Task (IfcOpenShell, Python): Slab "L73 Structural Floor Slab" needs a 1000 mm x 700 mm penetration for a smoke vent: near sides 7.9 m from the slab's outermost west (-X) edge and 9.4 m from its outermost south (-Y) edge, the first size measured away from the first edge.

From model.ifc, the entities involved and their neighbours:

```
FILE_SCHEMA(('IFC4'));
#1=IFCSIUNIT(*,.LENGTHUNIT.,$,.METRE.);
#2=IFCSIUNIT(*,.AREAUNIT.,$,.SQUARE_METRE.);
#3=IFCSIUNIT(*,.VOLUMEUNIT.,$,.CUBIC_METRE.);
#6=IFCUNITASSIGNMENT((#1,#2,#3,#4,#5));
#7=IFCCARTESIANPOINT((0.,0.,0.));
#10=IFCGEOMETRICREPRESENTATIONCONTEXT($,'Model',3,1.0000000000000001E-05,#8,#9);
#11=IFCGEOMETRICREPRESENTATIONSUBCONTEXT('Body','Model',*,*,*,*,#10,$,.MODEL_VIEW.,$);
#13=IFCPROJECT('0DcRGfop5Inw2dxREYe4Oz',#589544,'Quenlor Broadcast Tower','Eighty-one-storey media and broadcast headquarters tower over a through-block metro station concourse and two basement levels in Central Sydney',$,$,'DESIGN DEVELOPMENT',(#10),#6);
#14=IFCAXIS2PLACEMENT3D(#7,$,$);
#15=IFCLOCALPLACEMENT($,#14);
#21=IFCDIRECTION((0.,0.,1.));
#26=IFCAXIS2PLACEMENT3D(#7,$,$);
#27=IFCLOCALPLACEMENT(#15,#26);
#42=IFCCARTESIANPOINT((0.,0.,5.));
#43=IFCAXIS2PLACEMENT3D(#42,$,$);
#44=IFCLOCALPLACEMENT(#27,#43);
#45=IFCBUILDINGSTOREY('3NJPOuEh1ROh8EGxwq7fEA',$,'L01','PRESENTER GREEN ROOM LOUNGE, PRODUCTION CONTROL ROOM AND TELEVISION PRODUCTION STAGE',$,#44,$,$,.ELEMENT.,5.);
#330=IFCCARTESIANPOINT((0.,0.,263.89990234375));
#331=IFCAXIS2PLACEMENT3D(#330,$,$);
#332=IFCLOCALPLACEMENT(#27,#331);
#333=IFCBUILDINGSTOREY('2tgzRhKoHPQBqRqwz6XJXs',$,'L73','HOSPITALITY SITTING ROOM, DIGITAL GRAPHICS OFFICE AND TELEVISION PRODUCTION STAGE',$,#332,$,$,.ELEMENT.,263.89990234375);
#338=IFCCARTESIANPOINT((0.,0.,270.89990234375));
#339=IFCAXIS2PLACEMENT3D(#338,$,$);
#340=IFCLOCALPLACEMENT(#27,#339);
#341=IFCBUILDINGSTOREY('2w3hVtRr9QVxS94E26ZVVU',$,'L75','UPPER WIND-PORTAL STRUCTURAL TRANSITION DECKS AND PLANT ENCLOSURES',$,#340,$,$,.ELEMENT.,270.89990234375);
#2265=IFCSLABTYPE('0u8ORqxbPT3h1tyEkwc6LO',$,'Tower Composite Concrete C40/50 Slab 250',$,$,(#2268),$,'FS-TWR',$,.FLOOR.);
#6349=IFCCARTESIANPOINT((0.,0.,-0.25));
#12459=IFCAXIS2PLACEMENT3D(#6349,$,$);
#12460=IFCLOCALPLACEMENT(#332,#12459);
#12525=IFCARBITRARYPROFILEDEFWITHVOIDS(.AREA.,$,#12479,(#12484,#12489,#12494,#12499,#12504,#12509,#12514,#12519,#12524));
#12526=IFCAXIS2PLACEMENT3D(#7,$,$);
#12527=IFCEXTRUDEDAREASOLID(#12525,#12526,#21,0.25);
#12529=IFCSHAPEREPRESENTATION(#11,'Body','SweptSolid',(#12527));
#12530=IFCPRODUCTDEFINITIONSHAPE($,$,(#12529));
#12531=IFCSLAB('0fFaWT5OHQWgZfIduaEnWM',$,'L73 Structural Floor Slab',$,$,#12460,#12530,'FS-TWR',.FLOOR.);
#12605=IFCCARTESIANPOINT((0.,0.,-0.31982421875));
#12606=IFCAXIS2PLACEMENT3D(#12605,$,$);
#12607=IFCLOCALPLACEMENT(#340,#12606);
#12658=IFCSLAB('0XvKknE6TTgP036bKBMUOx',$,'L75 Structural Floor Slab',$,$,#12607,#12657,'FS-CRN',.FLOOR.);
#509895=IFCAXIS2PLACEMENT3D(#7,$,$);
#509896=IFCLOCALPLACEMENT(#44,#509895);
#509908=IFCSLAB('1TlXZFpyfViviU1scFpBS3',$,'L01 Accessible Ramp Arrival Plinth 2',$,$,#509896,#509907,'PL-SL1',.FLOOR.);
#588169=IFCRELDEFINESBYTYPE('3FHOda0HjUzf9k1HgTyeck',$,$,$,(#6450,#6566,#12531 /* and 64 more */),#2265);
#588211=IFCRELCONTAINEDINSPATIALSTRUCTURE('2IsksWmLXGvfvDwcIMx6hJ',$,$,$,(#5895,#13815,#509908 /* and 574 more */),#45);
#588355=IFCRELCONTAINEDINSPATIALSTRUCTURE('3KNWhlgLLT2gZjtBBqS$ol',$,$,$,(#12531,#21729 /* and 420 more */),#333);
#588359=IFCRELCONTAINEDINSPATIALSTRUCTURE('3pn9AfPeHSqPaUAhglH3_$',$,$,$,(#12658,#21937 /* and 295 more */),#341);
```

```python
import numpy as np
import ifcopenshell
import ifcopenshell.api.feature
import ifcopenshell.api.geometry
import ifcopenshell.api.root
import ifcopenshell.geom
import ifcopenshell.util.placement
import ifcopenshell.util.representation
import ifcopenshell.util.shape
import ifcopenshell.util.unit

model = ifcopenshell.open("model.ifc")
unit_scale = ifcopenshell.util.unit.calculate_unit_scale(model)
settings = ifcopenshell.geom.settings()


def volume(element):
    """Net volume in cubic metres, openings subtracted."""
    shape = ifcopenshell.geom.create_shape(settings, element)
    return ifcopenshell.util.shape.get_volume(shape.geometry)


slab = model.by_guid("0fFaWT5OHQWgZfIduaEnWM")
before = volume(slab)

# Extent in the slab's own axes, in metres. The edges named are its -X and -Y sides.
slab_shape = ifcopenshell.geom.create_shape(settings, slab)
vertices = ifcopenshell.util.shape.get_vertices(slab_shape.geometry)
x_min, y_min, bottom = vertices.min(axis=0)
top = vertices[:, 2].max()

opening = ifcopenshell.api.root.create_entity(model, ifc_class="IfcOpeningElement", name="Smoke vent opening", predefined_type="OPENING")
context = ifcopenshell.util.representation.get_context(model, "Model", "Body", "MODEL_VIEW")
width, depth = 1, 0.7
outline = [(0.0, 0.0), (width, 0.0), (width, depth), (0.0, depth), (0.0, 0.0)]
# Overshoot both faces by 50 mm so the cut is clean.
shape = ifcopenshell.api.geometry.add_slab_representation(
    model, context=context, depth=top - bottom + 0.1, polyline=outline
)
ifcopenshell.api.geometry.assign_representation(model, product=opening, representation=shape)

matrix = ifcopenshell.util.placement.get_local_placement(slab.ObjectPlacement)
matrix[:, 3] = matrix @ np.append(np.array([x_min + 7.9, y_min + 9.4, bottom - 0.05]) / unit_scale, 1.0)
ifcopenshell.api.geometry.edit_object_placement(model, product=opening, matrix=matrix, is_si=False)
ifcopenshell.api.feature.add_feature(model, feature=opening, element=slab)

after = volume(slab)

print(f"slab volume {before:.3f} -> {after:.3f} m3")

model.write("model-out.ifc")
```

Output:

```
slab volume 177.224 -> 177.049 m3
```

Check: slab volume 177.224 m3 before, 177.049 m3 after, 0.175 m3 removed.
